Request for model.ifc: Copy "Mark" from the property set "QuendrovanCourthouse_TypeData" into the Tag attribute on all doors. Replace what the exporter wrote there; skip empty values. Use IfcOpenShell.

First a look at what the model holds.

```python
import ifcopenshell
import ifcopenshell.util.element

model = ifcopenshell.open("model.ifc")
print(model.schema)
doors = model.by_type("IfcDoor")
print(len(doors), "doors")
for e in doors[:8]:
    source = ifcopenshell.util.element.get_pset(e, "QuendrovanCourthouse_TypeData", "Mark")
    target = e.Tag
    print(e.id(), repr(source), repr(target), sep=" | ")
```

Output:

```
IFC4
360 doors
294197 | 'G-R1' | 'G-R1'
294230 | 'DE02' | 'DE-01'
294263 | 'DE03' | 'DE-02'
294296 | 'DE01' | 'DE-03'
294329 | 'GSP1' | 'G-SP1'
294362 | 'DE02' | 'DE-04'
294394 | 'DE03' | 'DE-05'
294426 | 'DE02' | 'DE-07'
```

```python
import ifcopenshell
import ifcopenshell.util.element

model = ifcopenshell.open("model.ifc")

count = 0
for e in model.by_type("IfcDoor"):
    value = ifcopenshell.util.element.get_pset(e, "QuendrovanCourthouse_TypeData", "Mark")
    current = e.Tag
    if not value or not value.strip() or current == value:
        continue
    e.Tag = value
    count += 1

print(count, "doors updated")

model.write("model_edited.ifc")
```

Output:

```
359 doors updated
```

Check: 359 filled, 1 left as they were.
